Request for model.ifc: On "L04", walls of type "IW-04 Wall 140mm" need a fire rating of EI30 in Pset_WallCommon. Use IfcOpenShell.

First a look at what the model holds.

```python
import ifcopenshell
import ifcopenshell.util.element

model = ifcopenshell.open("model.ifc")
print(model.schema)
storey = next(s for s in model.by_type("IfcBuildingStorey") if s.Name == "L04")
walls = [e for e in ifcopenshell.util.element.get_decomposition(storey) if e.is_a("IfcWall")]
seen = {}
for e in walls:
    element_type = ifcopenshell.util.element.get_type(e)
    key = (element_type.Name if element_type != e and element_type else None, ifcopenshell.util.element.get_pset(e, "Pset_WallCommon", "FireRating"))
    seen[key] = seen.get(key, 0) + 1
for (name, value), count in sorted(seen.items(), key=str):
    print(count, "x", name, "|", value)
```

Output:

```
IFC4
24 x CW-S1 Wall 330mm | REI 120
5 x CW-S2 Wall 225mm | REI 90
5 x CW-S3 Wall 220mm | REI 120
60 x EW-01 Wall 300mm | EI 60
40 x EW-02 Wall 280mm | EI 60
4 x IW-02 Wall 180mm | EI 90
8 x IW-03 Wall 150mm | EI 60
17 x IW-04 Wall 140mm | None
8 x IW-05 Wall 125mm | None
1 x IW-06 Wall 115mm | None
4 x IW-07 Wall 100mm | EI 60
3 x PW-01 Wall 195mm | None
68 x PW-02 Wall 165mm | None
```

```python
import ifcopenshell
import ifcopenshell.api.pset
import ifcopenshell.util.element

model = ifcopenshell.open("model.ifc")

storey = next(s for s in model.by_type("IfcBuildingStorey") if s.Name == "L04")
walls = [e for e in ifcopenshell.util.element.get_decomposition(storey) if e.is_a("IfcWall")]

count = 0
for e in walls:
    element_type = ifcopenshell.util.element.get_type(e)
    if element_type in (None, e) or element_type.Name != "IW-04 Wall 140mm":
        continue
    # add_pset returns the element's existing set when there is one.
    pset = ifcopenshell.api.pset.add_pset(model, product=e, name="Pset_WallCommon")
    ifcopenshell.api.pset.edit_pset(model, pset=pset, properties={"FireRating": "EI30"})
    count += 1

print(count, "walls updated")

model.write("model_updated.ifc")
```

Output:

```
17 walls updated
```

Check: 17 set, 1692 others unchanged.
